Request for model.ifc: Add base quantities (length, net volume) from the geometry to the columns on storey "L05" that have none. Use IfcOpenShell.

First a look at what the model holds.

```python
import ifcopenshell
import ifcopenshell.util.element
import ifcopenshell.util.unit

model = ifcopenshell.open("model.ifc")
print(model.schema)
for unit_type in ("LENGTHUNIT", "AREAUNIT", "VOLUMEUNIT"):
    print(unit_type, ifcopenshell.util.unit.calculate_unit_scale(model, unit_type))
storey = next(s for s in model.by_type("IfcBuildingStorey") if s.Name == "L05")
columns = [e for e in ifcopenshell.util.element.get_decomposition(storey) if e.is_a("IfcColumn")]
for e in sorted(columns, key=lambda e: e.id()):
    print(e.id(), e.is_a(), e.Name, list(ifcopenshell.util.element.get_psets(e, qtos_only=True)), sep=" | ")
```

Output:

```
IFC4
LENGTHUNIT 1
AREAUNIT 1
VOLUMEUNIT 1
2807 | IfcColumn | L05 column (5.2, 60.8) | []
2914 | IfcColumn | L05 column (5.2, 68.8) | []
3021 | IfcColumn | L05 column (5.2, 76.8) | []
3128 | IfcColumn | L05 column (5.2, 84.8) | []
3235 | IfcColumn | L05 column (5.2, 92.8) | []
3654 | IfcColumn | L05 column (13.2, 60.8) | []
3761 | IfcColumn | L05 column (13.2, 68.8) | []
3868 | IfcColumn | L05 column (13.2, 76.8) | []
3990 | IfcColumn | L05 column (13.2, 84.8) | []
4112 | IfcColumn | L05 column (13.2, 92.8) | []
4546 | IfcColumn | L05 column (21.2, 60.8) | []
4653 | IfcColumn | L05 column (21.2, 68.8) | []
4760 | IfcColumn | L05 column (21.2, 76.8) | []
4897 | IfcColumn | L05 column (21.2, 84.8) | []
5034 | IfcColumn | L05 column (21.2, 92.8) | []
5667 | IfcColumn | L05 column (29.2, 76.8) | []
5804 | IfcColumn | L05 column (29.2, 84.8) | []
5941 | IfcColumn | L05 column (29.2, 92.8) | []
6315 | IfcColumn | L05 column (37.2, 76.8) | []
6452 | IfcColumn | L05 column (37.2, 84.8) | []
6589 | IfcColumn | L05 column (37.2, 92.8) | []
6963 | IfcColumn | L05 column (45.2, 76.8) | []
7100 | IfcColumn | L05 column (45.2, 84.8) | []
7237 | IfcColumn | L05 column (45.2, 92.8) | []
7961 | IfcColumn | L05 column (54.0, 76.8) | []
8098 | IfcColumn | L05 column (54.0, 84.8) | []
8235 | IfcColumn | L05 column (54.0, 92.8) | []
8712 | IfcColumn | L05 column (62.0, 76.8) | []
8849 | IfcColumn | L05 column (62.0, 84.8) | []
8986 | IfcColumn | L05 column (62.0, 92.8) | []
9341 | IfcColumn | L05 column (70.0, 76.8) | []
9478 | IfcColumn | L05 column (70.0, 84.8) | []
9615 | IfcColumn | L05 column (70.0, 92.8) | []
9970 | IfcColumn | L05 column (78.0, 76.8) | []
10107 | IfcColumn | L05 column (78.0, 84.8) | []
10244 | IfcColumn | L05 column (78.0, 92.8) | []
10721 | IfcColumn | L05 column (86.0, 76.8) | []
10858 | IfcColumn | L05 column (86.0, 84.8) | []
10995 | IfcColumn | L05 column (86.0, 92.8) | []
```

```python
import ifcopenshell
import ifcopenshell.api.pset
import ifcopenshell.geom
import ifcopenshell.util.element
import ifcopenshell.util.shape
import ifcopenshell.util.unit

model = ifcopenshell.open("model.ifc")
unit_scale = ifcopenshell.util.unit.calculate_unit_scale(model)
volume_scale = ifcopenshell.util.unit.calculate_unit_scale(model, "VOLUMEUNIT")
settings = ifcopenshell.geom.settings()

storey = next(s for s in model.by_type("IfcBuildingStorey") if s.Name == "L05")
columns = [e for e in ifcopenshell.util.element.get_decomposition(storey) if e.is_a("IfcColumn")]

for e in sorted(columns, key=lambda e: e.id()):
    if ifcopenshell.util.element.get_psets(e, qtos_only=True, should_inherit=False):
        continue
    # Geometry comes back in metres, in the element's own axes.
    shape = ifcopenshell.geom.create_shape(settings, e)
    values = {
        "Length": ifcopenshell.util.shape.get_z(shape.geometry) / unit_scale,
        "NetVolume": ifcopenshell.util.shape.get_volume(shape.geometry) / volume_scale,
    }
    qto = ifcopenshell.api.pset.add_qto(model, product=e, name="Qto_ColumnBaseQuantities")
    ifcopenshell.api.pset.edit_qto(model, qto=qto, properties=values)
    print(e.id(), {k: round(v, 3) for k, v in values.items()})

model.write("model_rev.ifc")
```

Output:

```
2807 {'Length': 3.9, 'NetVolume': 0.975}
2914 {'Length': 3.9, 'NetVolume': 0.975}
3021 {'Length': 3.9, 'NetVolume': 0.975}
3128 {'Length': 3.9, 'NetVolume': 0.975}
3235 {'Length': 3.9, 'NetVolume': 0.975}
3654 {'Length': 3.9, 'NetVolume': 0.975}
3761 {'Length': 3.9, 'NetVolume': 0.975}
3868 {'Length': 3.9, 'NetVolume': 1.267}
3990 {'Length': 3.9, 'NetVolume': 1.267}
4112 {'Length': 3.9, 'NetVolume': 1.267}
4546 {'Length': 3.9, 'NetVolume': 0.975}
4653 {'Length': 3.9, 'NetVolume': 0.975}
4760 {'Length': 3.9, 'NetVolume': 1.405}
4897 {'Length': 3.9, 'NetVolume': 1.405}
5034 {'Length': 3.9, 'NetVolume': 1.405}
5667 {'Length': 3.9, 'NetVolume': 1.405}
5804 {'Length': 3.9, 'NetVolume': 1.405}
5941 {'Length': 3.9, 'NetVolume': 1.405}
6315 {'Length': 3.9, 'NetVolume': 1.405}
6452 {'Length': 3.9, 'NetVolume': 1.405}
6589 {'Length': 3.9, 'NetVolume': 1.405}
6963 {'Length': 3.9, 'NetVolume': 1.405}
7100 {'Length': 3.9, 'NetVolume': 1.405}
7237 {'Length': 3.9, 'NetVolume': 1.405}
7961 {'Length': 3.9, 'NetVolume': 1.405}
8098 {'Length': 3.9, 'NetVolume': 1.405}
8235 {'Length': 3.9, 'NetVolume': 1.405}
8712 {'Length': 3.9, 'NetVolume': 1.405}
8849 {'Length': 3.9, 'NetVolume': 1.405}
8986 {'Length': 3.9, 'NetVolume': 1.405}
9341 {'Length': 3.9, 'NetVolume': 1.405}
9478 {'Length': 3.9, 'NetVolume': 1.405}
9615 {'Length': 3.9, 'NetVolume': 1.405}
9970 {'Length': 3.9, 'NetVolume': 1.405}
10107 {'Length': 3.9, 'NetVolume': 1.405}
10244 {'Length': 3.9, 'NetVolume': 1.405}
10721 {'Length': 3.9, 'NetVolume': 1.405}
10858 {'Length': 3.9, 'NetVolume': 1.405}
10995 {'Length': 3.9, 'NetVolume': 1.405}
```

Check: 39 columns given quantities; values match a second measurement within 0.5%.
